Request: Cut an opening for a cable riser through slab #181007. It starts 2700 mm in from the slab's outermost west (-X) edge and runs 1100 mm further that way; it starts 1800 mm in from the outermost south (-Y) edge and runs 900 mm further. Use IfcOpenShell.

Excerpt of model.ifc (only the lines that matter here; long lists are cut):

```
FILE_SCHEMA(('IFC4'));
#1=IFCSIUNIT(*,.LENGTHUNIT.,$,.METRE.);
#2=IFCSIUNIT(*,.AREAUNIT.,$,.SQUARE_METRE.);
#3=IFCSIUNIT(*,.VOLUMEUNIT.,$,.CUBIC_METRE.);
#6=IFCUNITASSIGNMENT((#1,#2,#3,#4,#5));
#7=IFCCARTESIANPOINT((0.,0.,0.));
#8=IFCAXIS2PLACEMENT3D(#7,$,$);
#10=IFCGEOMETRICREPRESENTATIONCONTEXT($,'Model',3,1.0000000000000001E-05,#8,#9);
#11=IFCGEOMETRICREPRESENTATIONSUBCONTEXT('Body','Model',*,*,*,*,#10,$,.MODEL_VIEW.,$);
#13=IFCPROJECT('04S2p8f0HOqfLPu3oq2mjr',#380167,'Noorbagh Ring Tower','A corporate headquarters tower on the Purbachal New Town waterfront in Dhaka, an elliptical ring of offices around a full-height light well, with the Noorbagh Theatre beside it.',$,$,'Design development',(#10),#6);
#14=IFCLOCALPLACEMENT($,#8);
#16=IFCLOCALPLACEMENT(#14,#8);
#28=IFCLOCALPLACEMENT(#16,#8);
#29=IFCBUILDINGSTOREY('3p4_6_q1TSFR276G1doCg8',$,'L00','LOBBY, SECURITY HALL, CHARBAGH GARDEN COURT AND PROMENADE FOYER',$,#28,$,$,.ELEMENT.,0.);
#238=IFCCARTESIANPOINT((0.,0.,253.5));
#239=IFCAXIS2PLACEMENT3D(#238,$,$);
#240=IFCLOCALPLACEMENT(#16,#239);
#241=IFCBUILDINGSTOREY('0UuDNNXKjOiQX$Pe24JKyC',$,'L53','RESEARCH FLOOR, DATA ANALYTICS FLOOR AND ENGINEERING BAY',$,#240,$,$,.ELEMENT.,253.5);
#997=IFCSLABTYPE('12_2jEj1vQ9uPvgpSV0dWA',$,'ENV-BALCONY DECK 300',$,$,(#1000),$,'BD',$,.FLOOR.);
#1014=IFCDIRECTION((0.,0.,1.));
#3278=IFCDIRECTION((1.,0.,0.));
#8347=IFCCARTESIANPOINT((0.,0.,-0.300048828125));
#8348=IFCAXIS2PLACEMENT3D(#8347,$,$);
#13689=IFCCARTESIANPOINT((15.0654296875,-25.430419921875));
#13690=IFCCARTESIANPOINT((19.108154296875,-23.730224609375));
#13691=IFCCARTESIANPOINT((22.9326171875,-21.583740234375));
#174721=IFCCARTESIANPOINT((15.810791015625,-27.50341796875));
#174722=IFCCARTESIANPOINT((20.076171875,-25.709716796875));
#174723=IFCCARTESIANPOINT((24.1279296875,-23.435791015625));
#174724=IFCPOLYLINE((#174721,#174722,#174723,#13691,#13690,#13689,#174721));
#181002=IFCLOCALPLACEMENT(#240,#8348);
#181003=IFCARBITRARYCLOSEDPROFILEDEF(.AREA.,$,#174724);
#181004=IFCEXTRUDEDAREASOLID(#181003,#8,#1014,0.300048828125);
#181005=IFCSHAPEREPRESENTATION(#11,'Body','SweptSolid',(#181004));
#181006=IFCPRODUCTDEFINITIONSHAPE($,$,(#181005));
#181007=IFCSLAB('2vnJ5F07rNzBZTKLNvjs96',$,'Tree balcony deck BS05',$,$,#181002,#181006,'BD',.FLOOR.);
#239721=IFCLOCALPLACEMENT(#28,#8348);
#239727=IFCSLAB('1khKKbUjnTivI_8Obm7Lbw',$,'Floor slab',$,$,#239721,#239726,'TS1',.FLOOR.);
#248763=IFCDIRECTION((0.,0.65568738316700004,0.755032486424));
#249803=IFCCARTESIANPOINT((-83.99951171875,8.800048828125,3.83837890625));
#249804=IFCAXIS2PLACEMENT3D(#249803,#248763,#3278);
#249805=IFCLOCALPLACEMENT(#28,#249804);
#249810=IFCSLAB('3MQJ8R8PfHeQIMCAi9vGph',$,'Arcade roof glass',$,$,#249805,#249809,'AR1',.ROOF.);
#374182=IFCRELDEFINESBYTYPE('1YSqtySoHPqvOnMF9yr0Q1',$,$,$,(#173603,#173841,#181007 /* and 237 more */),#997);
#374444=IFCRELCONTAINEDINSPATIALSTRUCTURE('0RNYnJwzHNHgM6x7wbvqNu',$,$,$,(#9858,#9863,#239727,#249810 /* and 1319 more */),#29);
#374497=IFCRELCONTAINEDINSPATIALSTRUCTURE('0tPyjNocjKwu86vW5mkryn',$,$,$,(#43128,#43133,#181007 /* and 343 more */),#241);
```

```python
import numpy as np
import ifcopenshell
import ifcopenshell.api.feature
import ifcopenshell.api.geometry
import ifcopenshell.api.root
import ifcopenshell.geom
import ifcopenshell.util.placement
import ifcopenshell.util.representation
import ifcopenshell.util.shape
import ifcopenshell.util.unit

model = ifcopenshell.open("model.ifc")
unit_scale = ifcopenshell.util.unit.calculate_unit_scale(model)
settings = ifcopenshell.geom.settings()


def volume(element):
    """Net volume in cubic metres, openings subtracted."""
    shape = ifcopenshell.geom.create_shape(settings, element)
    return ifcopenshell.util.shape.get_volume(shape.geometry)


slab = model.by_guid("2vnJ5F07rNzBZTKLNvjs96")
before = volume(slab)

# Extent in the slab's own axes, in metres. The edges named are its -X and -Y sides.
slab_shape = ifcopenshell.geom.create_shape(settings, slab)
vertices = ifcopenshell.util.shape.get_vertices(slab_shape.geometry)
x_min, y_min, bottom = vertices.min(axis=0)
top = vertices[:, 2].max()

opening = ifcopenshell.api.root.create_entity(model, ifc_class="IfcOpeningElement", name="Cable riser opening", predefined_type="OPENING")
context = ifcopenshell.util.representation.get_context(model, "Model", "Body", "MODEL_VIEW")
width, depth = 1.1, 0.9
outline = [(0.0, 0.0), (width, 0.0), (width, depth), (0.0, depth), (0.0, 0.0)]
# Overshoot both faces by 50 mm so the cut is clean.
shape = ifcopenshell.api.geometry.add_slab_representation(
    model, context=context, depth=top - bottom + 0.1, polyline=outline
)
ifcopenshell.api.geometry.assign_representation(model, product=opening, representation=shape)

matrix = ifcopenshell.util.placement.get_local_placement(slab.ObjectPlacement)
matrix[:, 3] = matrix @ np.append(np.array([x_min + 2.7, y_min + 1.8, bottom - 0.05]) / unit_scale, 1.0)
ifcopenshell.api.geometry.edit_object_placement(model, product=opening, matrix=matrix, is_si=False)
ifcopenshell.api.feature.add_feature(model, feature=opening, element=slab)

after = volume(slab)

print(f"slab volume {before:.3f} -> {after:.3f} m3")

model.write("model-out.ifc")
```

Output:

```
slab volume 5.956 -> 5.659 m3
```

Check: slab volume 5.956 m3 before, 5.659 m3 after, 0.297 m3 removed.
